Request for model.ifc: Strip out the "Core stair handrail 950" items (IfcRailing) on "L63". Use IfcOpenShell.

First a look at what the model holds.

```python
import ifcopenshell
import ifcopenshell.util.element

model = ifcopenshell.open("model.ifc")
print(model.schema)
storey = next(s for s in model.by_type("IfcBuildingStorey") if s.Name == "L63")
railings = [e for e in ifcopenshell.util.element.get_decomposition(storey) if e.is_a("IfcRailing")]
seen = {}
for e in railings:
    element_type = ifcopenshell.util.element.get_type(e)
    name = element_type.Name if element_type not in (None, e) else None
    seen[name] = seen.get(name, 0) + 1
for name, count in sorted(seen.items(), key=str):
    print(count, "x", name)
```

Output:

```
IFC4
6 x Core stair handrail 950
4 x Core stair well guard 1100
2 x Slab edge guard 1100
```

```python
import ifcopenshell
import ifcopenshell.api.root
import ifcopenshell.util.element

model = ifcopenshell.open("model.ifc")

storey = next(s for s in model.by_type("IfcBuildingStorey") if s.Name == "L63")
railings = [e for e in ifcopenshell.util.element.get_decomposition(storey) if e.is_a("IfcRailing")]
targets = [e for e in railings if (t := ifcopenshell.util.element.get_type(e)) not in (None, e) and t.Name == "Core stair handrail 950"]

for e in targets:
    ifcopenshell.api.root.remove_product(model, product=e)
print(len(targets), "removed")

model.write("model_v2.ifc")
```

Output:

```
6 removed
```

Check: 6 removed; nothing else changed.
